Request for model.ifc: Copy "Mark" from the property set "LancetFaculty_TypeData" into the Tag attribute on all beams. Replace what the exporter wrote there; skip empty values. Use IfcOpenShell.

First a look at what the model holds.

```python
import ifcopenshell
import ifcopenshell.util.element

model = ifcopenshell.open("model.ifc")
print(model.schema)
beams = model.by_type("IfcBeam")
print(len(beams), "beams")
for e in beams[:8]:
    source = ifcopenshell.util.element.get_pset(e, "LancetFaculty_TypeData", "Mark")
    target = e.Tag
    print(e.id(), repr(source), repr(target), sep=" | ")
```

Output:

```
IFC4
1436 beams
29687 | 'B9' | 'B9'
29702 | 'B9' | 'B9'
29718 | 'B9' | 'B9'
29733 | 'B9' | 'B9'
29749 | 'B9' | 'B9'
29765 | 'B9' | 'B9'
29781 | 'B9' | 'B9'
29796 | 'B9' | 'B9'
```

```python
import ifcopenshell
import ifcopenshell.util.element

model = ifcopenshell.open("model.ifc")

count = 0
for e in model.by_type("IfcBeam"):
    value = ifcopenshell.util.element.get_pset(e, "LancetFaculty_TypeData", "Mark")
    current = e.Tag
    if not value or not value.strip() or current == value:
        continue
    e.Tag = value
    count += 1

print(count, "beams updated")

model.write("model_v2.ifc")
```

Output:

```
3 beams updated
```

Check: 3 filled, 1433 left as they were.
